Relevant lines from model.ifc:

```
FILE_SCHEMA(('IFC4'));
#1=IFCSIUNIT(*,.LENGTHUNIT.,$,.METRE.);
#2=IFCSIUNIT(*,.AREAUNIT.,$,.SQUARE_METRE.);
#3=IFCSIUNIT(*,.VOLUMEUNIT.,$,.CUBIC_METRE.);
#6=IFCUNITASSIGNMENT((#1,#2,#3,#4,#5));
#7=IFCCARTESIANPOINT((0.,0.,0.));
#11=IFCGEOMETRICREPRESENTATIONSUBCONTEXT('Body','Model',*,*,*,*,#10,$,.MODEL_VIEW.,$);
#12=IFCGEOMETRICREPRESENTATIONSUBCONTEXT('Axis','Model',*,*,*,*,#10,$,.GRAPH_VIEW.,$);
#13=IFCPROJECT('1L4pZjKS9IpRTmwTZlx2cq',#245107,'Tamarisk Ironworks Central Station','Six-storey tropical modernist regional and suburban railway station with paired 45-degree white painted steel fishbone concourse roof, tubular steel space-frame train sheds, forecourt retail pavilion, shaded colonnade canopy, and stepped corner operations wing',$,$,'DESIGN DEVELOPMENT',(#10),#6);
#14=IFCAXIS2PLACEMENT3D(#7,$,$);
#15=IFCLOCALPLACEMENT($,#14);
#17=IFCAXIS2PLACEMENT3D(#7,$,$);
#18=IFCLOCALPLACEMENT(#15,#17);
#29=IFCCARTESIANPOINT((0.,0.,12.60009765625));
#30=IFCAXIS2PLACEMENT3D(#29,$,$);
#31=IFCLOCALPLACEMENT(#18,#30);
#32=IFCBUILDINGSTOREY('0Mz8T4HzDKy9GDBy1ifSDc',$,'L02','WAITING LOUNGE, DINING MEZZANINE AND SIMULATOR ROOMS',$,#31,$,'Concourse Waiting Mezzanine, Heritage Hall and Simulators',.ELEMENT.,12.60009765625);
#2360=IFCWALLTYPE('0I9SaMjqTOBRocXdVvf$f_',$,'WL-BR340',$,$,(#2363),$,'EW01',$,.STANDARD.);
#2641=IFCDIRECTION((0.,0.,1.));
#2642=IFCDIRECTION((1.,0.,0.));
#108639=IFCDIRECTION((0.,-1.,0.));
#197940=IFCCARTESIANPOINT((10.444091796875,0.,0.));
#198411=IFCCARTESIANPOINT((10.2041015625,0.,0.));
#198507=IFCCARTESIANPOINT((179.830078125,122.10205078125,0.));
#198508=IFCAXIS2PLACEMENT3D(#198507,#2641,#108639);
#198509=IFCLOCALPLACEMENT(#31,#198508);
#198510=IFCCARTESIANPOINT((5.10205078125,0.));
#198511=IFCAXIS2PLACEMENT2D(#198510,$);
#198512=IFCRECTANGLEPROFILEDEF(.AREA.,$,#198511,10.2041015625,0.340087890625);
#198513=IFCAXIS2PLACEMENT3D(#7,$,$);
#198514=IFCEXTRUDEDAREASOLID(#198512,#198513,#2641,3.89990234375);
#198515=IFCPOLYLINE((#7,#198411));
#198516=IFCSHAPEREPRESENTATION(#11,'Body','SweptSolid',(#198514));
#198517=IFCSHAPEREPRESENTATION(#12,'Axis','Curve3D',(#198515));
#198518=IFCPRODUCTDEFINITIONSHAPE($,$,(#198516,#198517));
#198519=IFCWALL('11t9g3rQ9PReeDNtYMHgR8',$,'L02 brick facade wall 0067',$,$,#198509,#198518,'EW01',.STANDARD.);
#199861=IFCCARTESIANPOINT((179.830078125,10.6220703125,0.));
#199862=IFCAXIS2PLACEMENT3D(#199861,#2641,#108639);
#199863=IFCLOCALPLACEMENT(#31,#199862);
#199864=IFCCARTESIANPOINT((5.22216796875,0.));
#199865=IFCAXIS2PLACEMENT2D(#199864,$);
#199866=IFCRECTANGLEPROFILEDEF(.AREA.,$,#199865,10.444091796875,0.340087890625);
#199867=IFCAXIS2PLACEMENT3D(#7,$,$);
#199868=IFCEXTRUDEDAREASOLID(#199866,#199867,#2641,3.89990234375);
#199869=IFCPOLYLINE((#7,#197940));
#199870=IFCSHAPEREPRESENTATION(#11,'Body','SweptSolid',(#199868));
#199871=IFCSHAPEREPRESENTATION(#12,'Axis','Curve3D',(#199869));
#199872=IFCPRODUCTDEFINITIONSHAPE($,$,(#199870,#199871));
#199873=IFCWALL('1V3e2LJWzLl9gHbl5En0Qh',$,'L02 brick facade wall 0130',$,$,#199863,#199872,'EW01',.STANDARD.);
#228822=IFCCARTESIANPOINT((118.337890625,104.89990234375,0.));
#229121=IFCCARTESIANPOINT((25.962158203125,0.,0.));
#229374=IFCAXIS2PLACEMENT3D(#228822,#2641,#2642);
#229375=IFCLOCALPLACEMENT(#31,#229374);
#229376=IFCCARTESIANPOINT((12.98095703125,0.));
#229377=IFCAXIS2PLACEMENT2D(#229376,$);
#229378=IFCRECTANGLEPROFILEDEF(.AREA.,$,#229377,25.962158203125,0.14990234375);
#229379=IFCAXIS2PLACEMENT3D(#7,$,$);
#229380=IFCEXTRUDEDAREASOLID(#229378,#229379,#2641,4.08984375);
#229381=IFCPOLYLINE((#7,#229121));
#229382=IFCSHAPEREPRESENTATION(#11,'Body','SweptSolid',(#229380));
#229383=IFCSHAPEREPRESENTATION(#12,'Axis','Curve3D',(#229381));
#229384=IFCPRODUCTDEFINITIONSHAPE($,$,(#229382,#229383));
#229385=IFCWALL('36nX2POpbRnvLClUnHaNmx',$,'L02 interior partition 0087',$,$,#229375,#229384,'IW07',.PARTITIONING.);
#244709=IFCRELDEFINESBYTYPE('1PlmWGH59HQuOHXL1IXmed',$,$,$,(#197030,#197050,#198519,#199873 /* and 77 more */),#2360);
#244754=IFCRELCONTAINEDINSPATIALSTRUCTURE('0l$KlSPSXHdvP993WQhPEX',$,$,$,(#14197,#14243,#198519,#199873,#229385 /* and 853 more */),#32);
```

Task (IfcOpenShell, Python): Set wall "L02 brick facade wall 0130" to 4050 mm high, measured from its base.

```python
import ifcopenshell
import ifcopenshell.geom
import ifcopenshell.util.representation
import ifcopenshell.util.shape

model = ifcopenshell.open("model.ifc")
settings = ifcopenshell.geom.settings()


def volume(element):
    """Net volume in cubic metres, openings subtracted."""
    shape = ifcopenshell.geom.create_shape(settings, element)
    return ifcopenshell.util.shape.get_volume(shape.geometry)


wall = model.by_guid("1V3e2LJWzLl9gHbl5En0Qh")
before = volume(wall)

body = ifcopenshell.util.representation.get_representation(wall, "Model", "Body")
solid = body.Items[0]
old_height = solid.Depth
solid.Depth = 4.05
after = volume(wall)

print(f"height {old_height:g} -> {solid.Depth:g}, volume {before:.3f} -> {after:.3f} m3")

model.write("model_updated.ifc")
```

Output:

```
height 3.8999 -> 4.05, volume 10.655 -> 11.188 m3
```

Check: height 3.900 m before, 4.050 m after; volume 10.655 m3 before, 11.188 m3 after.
